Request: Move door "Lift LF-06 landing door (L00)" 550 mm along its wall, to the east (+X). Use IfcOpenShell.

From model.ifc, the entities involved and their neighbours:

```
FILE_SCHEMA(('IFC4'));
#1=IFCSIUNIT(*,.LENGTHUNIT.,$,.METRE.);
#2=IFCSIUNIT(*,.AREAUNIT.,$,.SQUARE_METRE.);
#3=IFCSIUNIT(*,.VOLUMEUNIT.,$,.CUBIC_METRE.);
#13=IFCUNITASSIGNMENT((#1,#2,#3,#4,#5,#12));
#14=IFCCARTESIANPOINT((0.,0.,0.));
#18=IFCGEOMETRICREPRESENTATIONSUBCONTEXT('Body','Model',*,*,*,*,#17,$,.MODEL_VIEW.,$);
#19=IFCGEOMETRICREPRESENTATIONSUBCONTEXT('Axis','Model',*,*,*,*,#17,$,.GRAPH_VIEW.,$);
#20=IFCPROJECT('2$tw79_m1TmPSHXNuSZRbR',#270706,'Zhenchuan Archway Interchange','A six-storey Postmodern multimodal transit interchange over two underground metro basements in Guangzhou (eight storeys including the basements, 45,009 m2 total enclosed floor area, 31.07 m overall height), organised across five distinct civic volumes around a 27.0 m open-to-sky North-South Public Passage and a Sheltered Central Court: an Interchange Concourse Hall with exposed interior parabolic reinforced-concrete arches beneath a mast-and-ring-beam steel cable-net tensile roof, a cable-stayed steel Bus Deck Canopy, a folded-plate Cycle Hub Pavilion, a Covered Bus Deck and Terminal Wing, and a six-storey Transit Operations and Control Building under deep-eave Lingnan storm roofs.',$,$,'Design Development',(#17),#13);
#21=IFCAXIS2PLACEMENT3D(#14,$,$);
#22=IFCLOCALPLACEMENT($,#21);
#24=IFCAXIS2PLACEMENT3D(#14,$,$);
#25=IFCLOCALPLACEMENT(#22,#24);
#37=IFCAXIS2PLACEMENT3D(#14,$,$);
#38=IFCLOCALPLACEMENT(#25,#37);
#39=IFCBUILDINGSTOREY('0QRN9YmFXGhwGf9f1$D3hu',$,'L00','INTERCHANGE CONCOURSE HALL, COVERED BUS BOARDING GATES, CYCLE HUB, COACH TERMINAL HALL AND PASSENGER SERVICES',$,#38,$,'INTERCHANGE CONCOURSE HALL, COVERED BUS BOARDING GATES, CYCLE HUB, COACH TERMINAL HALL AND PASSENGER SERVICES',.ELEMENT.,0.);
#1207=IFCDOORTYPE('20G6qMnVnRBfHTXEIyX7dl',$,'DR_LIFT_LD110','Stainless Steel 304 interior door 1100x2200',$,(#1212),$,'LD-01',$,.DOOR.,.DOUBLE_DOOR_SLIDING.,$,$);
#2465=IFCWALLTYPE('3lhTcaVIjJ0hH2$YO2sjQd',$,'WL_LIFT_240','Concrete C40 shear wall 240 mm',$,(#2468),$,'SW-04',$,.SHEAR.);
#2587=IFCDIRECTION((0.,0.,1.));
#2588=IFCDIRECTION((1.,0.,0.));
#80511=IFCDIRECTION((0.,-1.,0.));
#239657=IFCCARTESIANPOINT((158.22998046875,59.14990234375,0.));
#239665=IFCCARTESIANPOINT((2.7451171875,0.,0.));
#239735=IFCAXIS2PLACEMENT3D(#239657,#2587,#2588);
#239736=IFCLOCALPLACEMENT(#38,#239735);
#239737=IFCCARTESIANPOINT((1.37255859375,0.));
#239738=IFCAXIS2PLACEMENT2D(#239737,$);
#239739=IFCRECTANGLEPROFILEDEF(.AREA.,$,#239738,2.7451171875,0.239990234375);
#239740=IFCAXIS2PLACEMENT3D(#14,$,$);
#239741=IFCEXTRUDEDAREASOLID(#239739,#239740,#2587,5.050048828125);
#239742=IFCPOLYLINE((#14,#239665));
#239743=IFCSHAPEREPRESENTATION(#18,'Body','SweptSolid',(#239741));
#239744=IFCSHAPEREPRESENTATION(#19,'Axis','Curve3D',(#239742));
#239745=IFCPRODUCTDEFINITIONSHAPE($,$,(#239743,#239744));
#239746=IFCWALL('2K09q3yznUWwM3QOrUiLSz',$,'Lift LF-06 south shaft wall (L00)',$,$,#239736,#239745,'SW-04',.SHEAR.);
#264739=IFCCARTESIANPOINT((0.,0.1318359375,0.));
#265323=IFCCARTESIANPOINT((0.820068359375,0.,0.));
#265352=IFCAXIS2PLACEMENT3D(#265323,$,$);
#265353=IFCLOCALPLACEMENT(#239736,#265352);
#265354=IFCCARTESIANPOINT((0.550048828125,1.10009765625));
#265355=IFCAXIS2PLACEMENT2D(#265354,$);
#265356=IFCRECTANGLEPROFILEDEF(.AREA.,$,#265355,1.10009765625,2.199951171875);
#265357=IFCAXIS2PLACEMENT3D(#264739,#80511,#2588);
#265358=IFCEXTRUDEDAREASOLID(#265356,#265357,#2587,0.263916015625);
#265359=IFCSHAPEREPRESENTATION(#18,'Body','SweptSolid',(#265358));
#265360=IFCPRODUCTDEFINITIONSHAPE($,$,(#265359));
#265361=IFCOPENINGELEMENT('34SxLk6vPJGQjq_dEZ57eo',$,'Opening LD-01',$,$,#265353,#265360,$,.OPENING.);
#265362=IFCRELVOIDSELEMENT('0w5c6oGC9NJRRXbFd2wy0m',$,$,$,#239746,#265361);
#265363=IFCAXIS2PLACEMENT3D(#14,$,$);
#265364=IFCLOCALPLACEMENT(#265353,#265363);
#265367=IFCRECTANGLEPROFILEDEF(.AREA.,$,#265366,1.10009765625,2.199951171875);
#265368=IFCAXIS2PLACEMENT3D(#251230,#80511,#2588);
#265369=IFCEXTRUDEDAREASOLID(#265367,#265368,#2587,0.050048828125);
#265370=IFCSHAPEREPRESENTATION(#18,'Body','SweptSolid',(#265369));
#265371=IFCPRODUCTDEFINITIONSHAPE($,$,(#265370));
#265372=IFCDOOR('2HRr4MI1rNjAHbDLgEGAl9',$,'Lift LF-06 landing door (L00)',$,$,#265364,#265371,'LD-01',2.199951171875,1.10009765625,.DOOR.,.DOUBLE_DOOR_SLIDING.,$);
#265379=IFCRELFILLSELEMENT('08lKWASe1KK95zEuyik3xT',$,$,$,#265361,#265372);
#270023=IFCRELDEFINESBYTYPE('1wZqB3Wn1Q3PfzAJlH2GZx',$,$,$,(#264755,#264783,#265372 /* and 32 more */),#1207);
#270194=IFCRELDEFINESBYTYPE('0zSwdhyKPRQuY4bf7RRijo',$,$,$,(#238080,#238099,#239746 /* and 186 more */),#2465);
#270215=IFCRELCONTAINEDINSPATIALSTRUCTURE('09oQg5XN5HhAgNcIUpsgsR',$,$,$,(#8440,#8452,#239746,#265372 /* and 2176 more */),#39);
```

```python
import ifcopenshell
import ifcopenshell.api.geometry
import ifcopenshell.util.placement
import ifcopenshell.util.unit

model = ifcopenshell.open("model.ifc")
unit_scale = ifcopenshell.util.unit.calculate_unit_scale(model)

door = model.by_id(265372)
opening = door.FillsVoids[0].RelatingOpeningElement
wall = opening.VoidsElements[0].RelatingBuildingElement

wall_matrix = ifcopenshell.util.placement.get_local_placement(wall.ObjectPlacement)
shift = wall_matrix[:3, 0] * 0.55 / unit_scale
before = ifcopenshell.util.placement.get_local_placement(door.ObjectPlacement)[:3, 3].copy()

# The door is placed relative to its opening, so it follows when the opening moves.
matrix = ifcopenshell.util.placement.get_local_placement(opening.ObjectPlacement)
matrix[:3, 3] += shift
ifcopenshell.api.geometry.edit_object_placement(
    model, product=opening, matrix=matrix, is_si=False, should_transform_children=True
)

after = ifcopenshell.util.placement.get_local_placement(door.ObjectPlacement)[:3, 3]
print("door moved by", (after - before).round(3) + 0.0)

model.write("model_updated.ifc")
```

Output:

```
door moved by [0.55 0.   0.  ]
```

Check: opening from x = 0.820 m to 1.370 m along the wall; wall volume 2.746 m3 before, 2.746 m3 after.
